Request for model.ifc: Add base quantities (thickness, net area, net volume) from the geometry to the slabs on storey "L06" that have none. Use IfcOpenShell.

First a look at what the model holds.

```python
import ifcopenshell
import ifcopenshell.util.element
import ifcopenshell.util.unit

model = ifcopenshell.open("model.ifc")
print(model.schema)
for unit_type in ("LENGTHUNIT", "AREAUNIT", "VOLUMEUNIT"):
    print(unit_type, ifcopenshell.util.unit.calculate_unit_scale(model, unit_type))
storey = next(s for s in model.by_type("IfcBuildingStorey") if s.Name == "L06")
slabs = [e for e in ifcopenshell.util.element.get_decomposition(storey) if e.is_a("IfcSlab")]
for e in sorted(slabs, key=lambda e: e.id()):
    print(e.id(), e.is_a(), e.Name, list(ifcopenshell.util.element.get_psets(e, qtos_only=True)), sep=" | ")
```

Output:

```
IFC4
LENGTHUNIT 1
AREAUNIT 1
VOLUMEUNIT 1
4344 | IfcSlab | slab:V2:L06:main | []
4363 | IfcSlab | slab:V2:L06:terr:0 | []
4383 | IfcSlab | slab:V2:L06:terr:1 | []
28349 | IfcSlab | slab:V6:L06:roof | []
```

```python
import ifcopenshell
import ifcopenshell.api.pset
import ifcopenshell.geom
import ifcopenshell.util.element
import ifcopenshell.util.shape
import ifcopenshell.util.unit

model = ifcopenshell.open("model.ifc")
unit_scale = ifcopenshell.util.unit.calculate_unit_scale(model)
area_scale = ifcopenshell.util.unit.calculate_unit_scale(model, "AREAUNIT")
volume_scale = ifcopenshell.util.unit.calculate_unit_scale(model, "VOLUMEUNIT")
settings = ifcopenshell.geom.settings()

storey = next(s for s in model.by_type("IfcBuildingStorey") if s.Name == "L06")
slabs = [e for e in ifcopenshell.util.element.get_decomposition(storey) if e.is_a("IfcSlab")]

for e in sorted(slabs, key=lambda e: e.id()):
    if ifcopenshell.util.element.get_psets(e, qtos_only=True, should_inherit=False):
        continue
    # Geometry comes back in metres, in the element's own axes.
    shape = ifcopenshell.geom.create_shape(settings, e)
    values = {
        "Width": ifcopenshell.util.shape.get_z(shape.geometry) / unit_scale,
        "NetArea": ifcopenshell.util.shape.get_footprint_area(shape.geometry) / area_scale,
        "NetVolume": ifcopenshell.util.shape.get_volume(shape.geometry) / volume_scale,
    }
    qto = ifcopenshell.api.pset.add_qto(model, product=e, name="Qto_SlabBaseQuantities")
    ifcopenshell.api.pset.edit_qto(model, qto=qto, properties=values)
    print(e.id(), {k: round(v, 3) for k, v in values.items()})

model.write("model_updated.ifc")
```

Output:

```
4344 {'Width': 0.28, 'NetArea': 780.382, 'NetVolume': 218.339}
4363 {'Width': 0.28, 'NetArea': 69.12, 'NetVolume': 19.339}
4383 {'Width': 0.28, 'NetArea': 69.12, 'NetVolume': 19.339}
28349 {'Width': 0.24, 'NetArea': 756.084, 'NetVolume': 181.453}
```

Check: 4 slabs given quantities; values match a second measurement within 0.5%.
